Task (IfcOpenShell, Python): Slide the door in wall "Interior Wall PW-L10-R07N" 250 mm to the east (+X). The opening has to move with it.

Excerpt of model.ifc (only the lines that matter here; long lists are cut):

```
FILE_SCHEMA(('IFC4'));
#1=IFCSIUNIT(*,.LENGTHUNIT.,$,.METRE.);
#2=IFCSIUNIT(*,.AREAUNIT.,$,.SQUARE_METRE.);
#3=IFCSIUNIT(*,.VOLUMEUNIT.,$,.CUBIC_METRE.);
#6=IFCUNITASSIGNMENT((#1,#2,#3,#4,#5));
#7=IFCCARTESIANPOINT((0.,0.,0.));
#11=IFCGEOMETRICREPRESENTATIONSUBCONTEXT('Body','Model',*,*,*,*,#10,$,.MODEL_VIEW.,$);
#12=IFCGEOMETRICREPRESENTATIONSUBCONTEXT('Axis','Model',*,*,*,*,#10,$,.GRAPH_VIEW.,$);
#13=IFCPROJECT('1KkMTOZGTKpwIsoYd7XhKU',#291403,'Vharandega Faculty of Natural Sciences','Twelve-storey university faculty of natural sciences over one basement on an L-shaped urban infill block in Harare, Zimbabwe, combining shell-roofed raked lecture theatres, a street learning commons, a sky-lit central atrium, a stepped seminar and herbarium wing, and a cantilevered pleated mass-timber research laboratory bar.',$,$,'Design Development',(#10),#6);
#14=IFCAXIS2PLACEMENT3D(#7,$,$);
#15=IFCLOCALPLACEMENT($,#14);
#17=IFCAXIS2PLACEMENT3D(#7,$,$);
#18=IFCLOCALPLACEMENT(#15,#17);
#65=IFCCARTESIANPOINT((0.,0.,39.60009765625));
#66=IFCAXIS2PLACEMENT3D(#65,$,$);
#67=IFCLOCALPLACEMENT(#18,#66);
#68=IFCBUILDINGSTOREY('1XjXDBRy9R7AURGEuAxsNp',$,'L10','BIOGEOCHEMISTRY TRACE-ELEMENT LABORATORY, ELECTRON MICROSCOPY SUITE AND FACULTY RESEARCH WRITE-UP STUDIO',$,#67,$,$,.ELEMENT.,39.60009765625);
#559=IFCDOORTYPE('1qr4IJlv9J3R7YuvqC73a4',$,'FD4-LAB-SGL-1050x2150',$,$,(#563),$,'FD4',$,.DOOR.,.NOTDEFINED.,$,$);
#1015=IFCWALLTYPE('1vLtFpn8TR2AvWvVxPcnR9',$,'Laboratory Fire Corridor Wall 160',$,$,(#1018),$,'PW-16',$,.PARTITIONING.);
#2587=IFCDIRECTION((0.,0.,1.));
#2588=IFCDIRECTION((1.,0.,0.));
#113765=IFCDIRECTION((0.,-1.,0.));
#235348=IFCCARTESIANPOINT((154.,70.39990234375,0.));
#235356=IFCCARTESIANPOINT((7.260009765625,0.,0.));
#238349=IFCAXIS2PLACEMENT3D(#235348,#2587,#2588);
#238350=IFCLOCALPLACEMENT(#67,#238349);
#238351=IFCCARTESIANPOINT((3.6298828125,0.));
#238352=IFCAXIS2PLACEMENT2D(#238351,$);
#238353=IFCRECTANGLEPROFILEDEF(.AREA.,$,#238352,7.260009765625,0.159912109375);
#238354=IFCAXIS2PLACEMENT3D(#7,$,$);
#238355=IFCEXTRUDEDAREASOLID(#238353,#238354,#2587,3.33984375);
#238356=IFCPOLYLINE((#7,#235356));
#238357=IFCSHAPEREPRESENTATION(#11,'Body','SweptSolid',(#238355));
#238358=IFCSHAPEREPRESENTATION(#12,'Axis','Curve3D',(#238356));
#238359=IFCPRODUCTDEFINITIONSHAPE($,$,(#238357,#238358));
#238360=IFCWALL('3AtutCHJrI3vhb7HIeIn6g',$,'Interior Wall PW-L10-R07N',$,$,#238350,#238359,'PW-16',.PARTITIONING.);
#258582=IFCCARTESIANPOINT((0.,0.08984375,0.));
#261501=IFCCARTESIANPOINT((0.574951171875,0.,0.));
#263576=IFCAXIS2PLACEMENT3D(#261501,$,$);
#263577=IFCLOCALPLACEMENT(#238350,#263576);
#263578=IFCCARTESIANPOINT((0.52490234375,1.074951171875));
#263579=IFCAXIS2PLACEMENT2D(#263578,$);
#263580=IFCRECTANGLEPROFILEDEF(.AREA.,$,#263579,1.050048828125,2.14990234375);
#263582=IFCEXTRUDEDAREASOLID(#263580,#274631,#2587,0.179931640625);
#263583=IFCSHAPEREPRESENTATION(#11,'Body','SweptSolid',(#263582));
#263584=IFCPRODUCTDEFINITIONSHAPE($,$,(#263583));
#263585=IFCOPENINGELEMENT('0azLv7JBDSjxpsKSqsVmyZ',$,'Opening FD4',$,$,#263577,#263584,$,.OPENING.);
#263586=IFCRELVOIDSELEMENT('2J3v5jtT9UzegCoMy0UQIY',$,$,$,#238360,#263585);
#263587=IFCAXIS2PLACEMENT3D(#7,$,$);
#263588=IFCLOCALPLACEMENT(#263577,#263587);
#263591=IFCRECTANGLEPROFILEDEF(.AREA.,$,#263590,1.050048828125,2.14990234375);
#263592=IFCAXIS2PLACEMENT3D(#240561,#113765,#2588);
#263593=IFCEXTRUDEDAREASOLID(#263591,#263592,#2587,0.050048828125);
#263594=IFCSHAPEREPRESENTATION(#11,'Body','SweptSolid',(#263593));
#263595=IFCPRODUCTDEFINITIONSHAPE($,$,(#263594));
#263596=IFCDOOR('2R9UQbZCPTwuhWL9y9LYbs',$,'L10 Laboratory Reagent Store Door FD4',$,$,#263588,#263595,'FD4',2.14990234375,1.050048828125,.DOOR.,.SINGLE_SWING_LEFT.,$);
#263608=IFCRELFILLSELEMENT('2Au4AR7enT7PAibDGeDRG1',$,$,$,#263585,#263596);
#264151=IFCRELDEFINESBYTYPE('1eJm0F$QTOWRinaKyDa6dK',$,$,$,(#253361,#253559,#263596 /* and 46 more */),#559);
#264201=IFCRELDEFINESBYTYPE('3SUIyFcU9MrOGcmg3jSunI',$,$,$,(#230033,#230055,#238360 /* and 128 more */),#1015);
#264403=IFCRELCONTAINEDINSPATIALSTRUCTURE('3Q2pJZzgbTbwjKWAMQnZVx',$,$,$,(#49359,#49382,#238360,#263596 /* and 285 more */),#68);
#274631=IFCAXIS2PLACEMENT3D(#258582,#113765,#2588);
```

```python
import ifcopenshell
import ifcopenshell.api.geometry
import ifcopenshell.util.placement
import ifcopenshell.util.unit

model = ifcopenshell.open("model.ifc")
unit_scale = ifcopenshell.util.unit.calculate_unit_scale(model)

door = model.by_guid("2R9UQbZCPTwuhWL9y9LYbs")
opening = door.FillsVoids[0].RelatingOpeningElement
wall = opening.VoidsElements[0].RelatingBuildingElement

wall_matrix = ifcopenshell.util.placement.get_local_placement(wall.ObjectPlacement)
shift = wall_matrix[:3, 0] * 0.25 / unit_scale
before = ifcopenshell.util.placement.get_local_placement(door.ObjectPlacement)[:3, 3].copy()

# The door is placed relative to its opening, so it follows when the opening moves.
matrix = ifcopenshell.util.placement.get_local_placement(opening.ObjectPlacement)
matrix[:3, 3] += shift
ifcopenshell.api.geometry.edit_object_placement(
    model, product=opening, matrix=matrix, is_si=False, should_transform_children=True
)

after = ifcopenshell.util.placement.get_local_placement(door.ObjectPlacement)[:3, 3]
print("door moved by", (after - before).round(3) + 0.0)

model.write("model_v2.ifc")
```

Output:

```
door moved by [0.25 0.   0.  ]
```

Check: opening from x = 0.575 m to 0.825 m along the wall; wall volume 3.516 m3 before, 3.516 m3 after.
